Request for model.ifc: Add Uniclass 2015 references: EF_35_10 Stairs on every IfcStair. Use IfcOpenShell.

First a look at what the model holds.

```python
import ifcopenshell

model = ifcopenshell.open("model.ifc")
print(model.schema)
print("classifications:", [c.Name for c in model.by_type("IfcClassification")])
for ifc_class in ("IfcDoor", "IfcRoof", "IfcStair", "IfcWall", "IfcWindow"):
    print(ifc_class, len(model.by_type(ifc_class)))
```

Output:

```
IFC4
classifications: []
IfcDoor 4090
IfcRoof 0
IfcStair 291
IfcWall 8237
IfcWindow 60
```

```python
import ifcopenshell
import ifcopenshell.api.classification

model = ifcopenshell.open("model.ifc")

system = ifcopenshell.api.classification.add_classification(model, classification="Uniclass 2015")

codes = {
    "IfcStair": ("EF_35_10", "Stairs"),
}
for ifc_class, (code, name) in codes.items():
    products = model.by_type(ifc_class)
    ifcopenshell.api.classification.add_reference(
        model, products=products, classification=system, identification=code, name=name
    )
    print(code, len(products))

model.write("model_edited.ifc")
```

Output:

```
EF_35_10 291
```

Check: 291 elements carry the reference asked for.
